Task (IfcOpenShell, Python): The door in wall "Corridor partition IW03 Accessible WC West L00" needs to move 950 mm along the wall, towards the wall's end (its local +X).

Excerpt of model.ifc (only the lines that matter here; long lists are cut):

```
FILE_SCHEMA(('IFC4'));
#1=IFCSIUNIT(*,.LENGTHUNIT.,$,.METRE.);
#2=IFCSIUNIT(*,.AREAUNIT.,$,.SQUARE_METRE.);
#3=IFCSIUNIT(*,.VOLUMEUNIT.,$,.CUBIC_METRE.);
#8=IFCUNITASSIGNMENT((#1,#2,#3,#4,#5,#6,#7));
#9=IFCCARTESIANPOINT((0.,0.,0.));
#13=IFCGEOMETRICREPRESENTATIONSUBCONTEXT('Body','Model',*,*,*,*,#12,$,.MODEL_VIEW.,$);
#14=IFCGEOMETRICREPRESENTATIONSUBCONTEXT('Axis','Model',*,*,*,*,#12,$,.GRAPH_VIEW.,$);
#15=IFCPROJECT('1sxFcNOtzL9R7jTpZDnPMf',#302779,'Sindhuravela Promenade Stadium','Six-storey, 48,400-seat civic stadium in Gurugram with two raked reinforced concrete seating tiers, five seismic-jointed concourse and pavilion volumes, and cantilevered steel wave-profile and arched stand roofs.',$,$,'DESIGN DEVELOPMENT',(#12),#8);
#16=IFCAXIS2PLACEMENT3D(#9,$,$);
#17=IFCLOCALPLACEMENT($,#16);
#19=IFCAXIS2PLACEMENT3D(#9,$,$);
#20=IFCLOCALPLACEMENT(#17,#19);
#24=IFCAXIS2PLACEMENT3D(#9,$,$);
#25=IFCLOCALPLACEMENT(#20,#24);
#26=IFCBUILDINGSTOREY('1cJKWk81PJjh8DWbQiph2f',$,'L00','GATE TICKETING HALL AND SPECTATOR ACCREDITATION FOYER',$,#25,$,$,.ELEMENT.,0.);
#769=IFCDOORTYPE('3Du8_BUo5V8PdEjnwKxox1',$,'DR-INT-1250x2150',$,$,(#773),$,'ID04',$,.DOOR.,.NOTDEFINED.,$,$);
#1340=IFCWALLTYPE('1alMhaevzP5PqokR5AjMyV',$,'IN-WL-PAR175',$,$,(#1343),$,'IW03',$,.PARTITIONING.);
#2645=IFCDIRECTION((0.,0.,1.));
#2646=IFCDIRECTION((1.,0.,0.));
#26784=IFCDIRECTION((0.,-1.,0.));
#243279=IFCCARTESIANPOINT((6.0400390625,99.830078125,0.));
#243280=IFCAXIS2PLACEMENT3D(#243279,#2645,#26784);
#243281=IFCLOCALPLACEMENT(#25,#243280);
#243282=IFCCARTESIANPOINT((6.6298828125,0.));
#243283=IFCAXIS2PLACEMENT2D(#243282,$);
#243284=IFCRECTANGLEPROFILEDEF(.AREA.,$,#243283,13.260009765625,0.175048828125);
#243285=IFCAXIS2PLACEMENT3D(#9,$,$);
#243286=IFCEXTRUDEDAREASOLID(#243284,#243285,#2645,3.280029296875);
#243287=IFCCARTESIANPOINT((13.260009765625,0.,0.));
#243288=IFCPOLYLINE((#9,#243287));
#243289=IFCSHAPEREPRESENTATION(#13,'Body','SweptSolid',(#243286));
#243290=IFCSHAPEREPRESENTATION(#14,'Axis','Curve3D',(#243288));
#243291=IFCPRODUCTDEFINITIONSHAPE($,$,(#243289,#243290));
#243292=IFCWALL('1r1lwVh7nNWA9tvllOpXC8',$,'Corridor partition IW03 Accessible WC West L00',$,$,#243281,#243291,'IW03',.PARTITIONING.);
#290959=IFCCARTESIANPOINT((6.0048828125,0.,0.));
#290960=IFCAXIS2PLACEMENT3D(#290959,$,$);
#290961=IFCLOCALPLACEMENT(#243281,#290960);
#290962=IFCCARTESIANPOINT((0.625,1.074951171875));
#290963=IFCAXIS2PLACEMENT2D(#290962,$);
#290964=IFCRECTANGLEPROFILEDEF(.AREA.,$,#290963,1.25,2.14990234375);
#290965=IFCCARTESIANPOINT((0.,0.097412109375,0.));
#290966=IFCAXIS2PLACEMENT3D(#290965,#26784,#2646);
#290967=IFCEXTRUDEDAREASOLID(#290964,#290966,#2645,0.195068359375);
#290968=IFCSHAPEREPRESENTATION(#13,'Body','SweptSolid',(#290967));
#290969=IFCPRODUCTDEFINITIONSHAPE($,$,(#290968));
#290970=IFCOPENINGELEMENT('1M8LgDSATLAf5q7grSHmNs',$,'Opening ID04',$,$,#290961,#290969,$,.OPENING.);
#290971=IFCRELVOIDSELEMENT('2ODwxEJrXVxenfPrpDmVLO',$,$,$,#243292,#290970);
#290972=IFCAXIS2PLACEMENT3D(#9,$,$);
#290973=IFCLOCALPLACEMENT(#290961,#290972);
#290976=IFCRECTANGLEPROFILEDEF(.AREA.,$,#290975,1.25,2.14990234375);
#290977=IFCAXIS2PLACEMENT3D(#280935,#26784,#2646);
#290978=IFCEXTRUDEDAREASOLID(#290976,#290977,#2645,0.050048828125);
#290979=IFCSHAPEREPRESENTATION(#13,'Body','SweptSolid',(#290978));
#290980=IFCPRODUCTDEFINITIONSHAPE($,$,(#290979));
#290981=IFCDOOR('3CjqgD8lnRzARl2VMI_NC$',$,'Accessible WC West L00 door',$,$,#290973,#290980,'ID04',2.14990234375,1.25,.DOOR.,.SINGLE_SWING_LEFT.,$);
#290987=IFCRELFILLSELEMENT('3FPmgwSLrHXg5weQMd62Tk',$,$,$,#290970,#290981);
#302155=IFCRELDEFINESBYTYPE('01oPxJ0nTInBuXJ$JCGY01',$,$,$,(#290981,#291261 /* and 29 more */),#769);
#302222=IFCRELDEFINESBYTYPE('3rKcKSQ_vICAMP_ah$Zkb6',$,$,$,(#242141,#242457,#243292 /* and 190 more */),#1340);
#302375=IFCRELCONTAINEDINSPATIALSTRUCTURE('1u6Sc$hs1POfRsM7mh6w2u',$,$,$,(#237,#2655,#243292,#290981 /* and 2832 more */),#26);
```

```python
import ifcopenshell
import ifcopenshell.api.geometry
import ifcopenshell.util.placement

model = ifcopenshell.open("model.ifc")

door = model.by_id(290981)
opening = door.FillsVoids[0].RelatingOpeningElement
wall = opening.VoidsElements[0].RelatingBuildingElement

wall_matrix = ifcopenshell.util.placement.get_local_placement(wall.ObjectPlacement)
shift = wall_matrix[:3, 0] * 0.95
before = ifcopenshell.util.placement.get_local_placement(door.ObjectPlacement)[:3, 3].copy()

# The door is placed relative to its opening, so it follows when the opening moves.
matrix = ifcopenshell.util.placement.get_local_placement(opening.ObjectPlacement)
matrix[:3, 3] += shift
ifcopenshell.api.geometry.edit_object_placement(
    model, product=opening, matrix=matrix, is_si=False, should_transform_children=True
)

after = ifcopenshell.util.placement.get_local_placement(door.ObjectPlacement)[:3, 3]
print("door moved by", (after - before).round(3) + 0.0)

model.write("model_v2.ifc")
```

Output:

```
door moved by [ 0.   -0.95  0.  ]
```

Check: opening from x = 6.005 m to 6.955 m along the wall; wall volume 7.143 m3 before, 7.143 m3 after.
